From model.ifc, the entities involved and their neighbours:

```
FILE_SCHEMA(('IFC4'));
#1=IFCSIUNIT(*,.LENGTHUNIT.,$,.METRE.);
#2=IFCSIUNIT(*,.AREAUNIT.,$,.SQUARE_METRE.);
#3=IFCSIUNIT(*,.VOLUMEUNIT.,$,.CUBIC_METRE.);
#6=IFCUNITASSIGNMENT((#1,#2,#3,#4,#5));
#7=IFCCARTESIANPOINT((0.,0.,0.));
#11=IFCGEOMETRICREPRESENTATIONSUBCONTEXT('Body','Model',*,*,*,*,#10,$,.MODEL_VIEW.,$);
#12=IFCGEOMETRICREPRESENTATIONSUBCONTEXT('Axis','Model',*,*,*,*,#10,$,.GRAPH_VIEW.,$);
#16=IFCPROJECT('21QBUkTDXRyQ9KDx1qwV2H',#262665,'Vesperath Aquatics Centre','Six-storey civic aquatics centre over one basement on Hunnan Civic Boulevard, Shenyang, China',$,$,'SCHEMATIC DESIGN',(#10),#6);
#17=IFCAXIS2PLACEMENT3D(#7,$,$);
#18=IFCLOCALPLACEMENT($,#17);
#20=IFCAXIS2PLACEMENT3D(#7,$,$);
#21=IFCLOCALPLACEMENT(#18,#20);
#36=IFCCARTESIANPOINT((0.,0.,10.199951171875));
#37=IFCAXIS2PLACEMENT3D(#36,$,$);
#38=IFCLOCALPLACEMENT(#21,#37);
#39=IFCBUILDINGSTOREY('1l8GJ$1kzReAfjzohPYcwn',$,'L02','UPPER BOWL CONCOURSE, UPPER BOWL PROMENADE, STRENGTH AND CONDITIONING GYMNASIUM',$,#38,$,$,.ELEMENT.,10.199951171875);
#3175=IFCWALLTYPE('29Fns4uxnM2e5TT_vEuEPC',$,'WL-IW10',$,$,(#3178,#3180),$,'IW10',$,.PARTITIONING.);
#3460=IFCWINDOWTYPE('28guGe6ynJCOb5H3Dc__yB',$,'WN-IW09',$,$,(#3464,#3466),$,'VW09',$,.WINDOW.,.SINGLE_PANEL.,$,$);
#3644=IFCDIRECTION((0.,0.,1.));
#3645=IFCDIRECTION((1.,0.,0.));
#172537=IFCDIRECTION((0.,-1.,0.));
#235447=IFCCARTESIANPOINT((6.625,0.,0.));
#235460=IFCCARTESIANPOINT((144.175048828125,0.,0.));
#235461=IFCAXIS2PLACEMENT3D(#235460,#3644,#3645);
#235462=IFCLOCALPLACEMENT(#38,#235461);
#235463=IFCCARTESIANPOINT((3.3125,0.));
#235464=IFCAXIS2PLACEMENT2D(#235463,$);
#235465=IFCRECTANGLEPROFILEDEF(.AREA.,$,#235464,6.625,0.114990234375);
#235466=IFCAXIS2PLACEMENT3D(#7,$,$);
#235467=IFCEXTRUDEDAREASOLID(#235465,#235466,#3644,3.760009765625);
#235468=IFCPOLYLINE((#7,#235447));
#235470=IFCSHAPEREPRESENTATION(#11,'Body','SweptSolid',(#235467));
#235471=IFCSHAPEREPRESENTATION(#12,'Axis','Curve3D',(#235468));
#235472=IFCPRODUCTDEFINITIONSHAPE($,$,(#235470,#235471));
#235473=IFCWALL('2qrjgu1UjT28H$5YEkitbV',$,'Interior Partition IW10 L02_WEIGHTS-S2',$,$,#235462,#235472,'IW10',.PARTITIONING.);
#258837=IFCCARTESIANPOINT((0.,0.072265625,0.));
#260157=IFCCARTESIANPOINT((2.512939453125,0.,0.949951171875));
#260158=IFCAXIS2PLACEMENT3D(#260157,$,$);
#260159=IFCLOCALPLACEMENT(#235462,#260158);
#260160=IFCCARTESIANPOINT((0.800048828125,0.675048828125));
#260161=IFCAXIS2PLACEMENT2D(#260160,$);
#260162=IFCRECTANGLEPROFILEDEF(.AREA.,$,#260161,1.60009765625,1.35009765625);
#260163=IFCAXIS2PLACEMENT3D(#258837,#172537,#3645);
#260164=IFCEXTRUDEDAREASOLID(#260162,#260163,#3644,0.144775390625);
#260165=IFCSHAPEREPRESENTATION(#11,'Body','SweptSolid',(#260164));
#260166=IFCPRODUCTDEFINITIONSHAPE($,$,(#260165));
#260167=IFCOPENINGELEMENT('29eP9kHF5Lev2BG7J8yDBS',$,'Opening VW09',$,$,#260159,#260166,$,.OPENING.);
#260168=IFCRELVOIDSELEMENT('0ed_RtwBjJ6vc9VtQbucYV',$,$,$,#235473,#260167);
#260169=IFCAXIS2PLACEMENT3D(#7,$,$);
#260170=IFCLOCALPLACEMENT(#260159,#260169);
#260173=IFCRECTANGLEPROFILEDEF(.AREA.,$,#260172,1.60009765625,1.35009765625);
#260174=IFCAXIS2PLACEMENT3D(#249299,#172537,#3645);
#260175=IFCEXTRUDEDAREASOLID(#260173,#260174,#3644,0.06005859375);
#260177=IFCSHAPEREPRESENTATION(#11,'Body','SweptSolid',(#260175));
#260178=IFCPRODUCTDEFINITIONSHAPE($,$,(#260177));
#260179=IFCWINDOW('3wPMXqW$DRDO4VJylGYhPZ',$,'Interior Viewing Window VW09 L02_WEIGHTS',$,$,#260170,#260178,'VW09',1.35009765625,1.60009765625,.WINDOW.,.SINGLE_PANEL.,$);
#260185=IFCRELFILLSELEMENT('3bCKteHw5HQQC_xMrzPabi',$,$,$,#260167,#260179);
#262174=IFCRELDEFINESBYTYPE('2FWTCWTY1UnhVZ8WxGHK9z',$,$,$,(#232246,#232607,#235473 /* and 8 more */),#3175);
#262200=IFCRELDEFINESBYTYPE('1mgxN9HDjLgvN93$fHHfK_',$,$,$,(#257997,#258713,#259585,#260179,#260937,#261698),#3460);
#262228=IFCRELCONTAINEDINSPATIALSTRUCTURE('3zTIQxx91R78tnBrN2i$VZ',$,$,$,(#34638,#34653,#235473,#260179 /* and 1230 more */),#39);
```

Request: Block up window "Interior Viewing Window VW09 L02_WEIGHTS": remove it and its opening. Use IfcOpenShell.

```python
import ifcopenshell
import ifcopenshell.api.feature
import ifcopenshell.api.root
import ifcopenshell.geom
import ifcopenshell.util.shape

model = ifcopenshell.open("model.ifc")
settings = ifcopenshell.geom.settings()


def volume(element):
    """Net volume in cubic metres, openings subtracted."""
    shape = ifcopenshell.geom.create_shape(settings, element)
    return ifcopenshell.util.shape.get_volume(shape.geometry)


window = model.by_guid("3wPMXqW$DRDO4VJylGYhPZ")
opening = window.FillsVoids[0].RelatingOpeningElement
wall = opening.VoidsElements[0].RelatingBuildingElement
before = volume(wall)

ifcopenshell.api.root.remove_product(model, product=window)
ifcopenshell.api.feature.remove_feature(model, feature=opening)

after = volume(wall)

print(f"wall volume {before:.3f} -> {after:.3f} m3")

model.write("model-out.ifc")
```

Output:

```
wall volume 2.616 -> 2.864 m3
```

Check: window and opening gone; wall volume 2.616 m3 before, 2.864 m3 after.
